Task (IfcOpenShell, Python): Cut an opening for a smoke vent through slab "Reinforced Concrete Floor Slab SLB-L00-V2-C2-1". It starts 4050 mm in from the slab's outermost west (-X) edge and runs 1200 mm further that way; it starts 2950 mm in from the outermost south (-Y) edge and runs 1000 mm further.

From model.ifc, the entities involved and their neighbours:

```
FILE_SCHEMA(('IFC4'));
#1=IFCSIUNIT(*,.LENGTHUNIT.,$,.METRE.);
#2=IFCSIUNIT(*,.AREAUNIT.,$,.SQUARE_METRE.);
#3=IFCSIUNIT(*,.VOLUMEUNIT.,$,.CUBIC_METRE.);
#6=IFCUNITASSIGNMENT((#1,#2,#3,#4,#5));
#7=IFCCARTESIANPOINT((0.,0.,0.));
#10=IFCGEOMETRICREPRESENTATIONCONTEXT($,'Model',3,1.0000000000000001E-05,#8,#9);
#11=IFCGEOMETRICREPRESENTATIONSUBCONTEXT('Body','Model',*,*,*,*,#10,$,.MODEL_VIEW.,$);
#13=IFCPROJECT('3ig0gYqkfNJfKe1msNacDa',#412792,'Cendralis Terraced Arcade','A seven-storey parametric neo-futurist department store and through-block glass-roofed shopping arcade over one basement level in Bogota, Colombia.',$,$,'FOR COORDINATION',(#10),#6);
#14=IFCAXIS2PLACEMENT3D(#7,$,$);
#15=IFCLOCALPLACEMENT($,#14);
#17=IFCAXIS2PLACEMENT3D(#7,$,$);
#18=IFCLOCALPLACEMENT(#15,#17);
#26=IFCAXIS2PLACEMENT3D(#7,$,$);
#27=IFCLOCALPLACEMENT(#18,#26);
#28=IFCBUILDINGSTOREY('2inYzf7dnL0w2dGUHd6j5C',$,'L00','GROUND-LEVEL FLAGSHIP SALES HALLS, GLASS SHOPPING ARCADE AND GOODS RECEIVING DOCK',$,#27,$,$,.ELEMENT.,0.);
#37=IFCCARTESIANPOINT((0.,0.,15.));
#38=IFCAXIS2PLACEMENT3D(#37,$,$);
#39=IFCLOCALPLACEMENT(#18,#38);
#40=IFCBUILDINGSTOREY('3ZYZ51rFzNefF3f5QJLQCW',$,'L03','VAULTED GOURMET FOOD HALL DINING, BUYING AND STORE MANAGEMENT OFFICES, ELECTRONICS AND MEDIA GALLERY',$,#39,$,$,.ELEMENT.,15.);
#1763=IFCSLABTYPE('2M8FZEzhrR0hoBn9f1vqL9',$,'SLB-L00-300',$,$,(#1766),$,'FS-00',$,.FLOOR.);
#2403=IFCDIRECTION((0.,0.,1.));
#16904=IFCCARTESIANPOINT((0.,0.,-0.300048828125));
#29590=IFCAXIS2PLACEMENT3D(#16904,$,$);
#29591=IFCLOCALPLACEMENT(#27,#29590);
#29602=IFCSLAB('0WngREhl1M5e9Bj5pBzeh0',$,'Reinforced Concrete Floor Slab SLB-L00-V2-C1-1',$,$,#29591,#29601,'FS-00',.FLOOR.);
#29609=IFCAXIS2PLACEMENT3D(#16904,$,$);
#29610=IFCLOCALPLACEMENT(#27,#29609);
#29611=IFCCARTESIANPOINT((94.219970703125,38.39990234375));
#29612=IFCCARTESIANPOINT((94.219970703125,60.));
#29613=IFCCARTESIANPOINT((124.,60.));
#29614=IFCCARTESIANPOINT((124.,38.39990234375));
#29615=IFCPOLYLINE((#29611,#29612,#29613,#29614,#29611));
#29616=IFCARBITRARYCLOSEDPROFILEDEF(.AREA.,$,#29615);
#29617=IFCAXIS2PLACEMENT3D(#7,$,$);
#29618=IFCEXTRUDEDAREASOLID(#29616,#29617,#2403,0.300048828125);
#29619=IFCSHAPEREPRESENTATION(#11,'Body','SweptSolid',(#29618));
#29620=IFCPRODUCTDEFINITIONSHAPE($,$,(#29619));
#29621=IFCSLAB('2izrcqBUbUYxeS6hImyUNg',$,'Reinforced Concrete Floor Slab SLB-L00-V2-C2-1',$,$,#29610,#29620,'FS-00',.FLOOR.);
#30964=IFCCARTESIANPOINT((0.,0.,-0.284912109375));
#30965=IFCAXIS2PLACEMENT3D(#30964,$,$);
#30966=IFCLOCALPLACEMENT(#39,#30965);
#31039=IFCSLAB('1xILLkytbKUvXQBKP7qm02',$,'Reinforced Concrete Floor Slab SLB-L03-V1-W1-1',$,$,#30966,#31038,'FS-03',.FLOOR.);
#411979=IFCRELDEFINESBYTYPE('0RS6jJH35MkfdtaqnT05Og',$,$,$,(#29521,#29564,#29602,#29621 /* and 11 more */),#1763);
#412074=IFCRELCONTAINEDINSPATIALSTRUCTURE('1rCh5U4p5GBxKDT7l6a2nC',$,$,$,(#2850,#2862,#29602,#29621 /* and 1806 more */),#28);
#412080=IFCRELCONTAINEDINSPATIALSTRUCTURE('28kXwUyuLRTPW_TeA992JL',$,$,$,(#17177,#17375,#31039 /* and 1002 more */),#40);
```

```python
import numpy as np
import ifcopenshell
import ifcopenshell.api.feature
import ifcopenshell.api.geometry
import ifcopenshell.api.root
import ifcopenshell.geom
import ifcopenshell.util.placement
import ifcopenshell.util.representation
import ifcopenshell.util.shape
import ifcopenshell.util.unit

model = ifcopenshell.open("model.ifc")
unit_scale = ifcopenshell.util.unit.calculate_unit_scale(model)
settings = ifcopenshell.geom.settings()


def volume(element):
    """Net volume in cubic metres, openings subtracted."""
    shape = ifcopenshell.geom.create_shape(settings, element)
    return ifcopenshell.util.shape.get_volume(shape.geometry)


slab = model.by_guid("2izrcqBUbUYxeS6hImyUNg")
before = volume(slab)

# Extent in the slab's own axes, in metres. The edges named are its -X and -Y sides.
slab_shape = ifcopenshell.geom.create_shape(settings, slab)
vertices = ifcopenshell.util.shape.get_vertices(slab_shape.geometry)
x_min, y_min, bottom = vertices.min(axis=0)
top = vertices[:, 2].max()

opening = ifcopenshell.api.root.create_entity(model, ifc_class="IfcOpeningElement", name="Smoke vent opening", predefined_type="OPENING")
context = ifcopenshell.util.representation.get_context(model, "Model", "Body", "MODEL_VIEW")
width, depth = 1.2, 1
outline = [(0.0, 0.0), (width, 0.0), (width, depth), (0.0, depth), (0.0, 0.0)]
# Overshoot both faces by 50 mm so the cut is clean.
shape = ifcopenshell.api.geometry.add_slab_representation(
    model, context=context, depth=top - bottom + 0.1, polyline=outline
)
ifcopenshell.api.geometry.assign_representation(model, product=opening, representation=shape)

matrix = ifcopenshell.util.placement.get_local_placement(slab.ObjectPlacement)
matrix[:, 3] = matrix @ np.append(np.array([x_min + 4.05, y_min + 2.95, bottom - 0.05]) / unit_scale, 1.0)
ifcopenshell.api.geometry.edit_object_placement(model, product=opening, matrix=matrix, is_si=False)
ifcopenshell.api.feature.add_feature(model, feature=opening, element=slab)

after = volume(slab)

print(f"slab volume {before:.3f} -> {after:.3f} m3")

model.write("model_edited.ifc")
```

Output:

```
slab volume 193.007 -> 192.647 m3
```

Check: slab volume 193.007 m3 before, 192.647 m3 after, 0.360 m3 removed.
